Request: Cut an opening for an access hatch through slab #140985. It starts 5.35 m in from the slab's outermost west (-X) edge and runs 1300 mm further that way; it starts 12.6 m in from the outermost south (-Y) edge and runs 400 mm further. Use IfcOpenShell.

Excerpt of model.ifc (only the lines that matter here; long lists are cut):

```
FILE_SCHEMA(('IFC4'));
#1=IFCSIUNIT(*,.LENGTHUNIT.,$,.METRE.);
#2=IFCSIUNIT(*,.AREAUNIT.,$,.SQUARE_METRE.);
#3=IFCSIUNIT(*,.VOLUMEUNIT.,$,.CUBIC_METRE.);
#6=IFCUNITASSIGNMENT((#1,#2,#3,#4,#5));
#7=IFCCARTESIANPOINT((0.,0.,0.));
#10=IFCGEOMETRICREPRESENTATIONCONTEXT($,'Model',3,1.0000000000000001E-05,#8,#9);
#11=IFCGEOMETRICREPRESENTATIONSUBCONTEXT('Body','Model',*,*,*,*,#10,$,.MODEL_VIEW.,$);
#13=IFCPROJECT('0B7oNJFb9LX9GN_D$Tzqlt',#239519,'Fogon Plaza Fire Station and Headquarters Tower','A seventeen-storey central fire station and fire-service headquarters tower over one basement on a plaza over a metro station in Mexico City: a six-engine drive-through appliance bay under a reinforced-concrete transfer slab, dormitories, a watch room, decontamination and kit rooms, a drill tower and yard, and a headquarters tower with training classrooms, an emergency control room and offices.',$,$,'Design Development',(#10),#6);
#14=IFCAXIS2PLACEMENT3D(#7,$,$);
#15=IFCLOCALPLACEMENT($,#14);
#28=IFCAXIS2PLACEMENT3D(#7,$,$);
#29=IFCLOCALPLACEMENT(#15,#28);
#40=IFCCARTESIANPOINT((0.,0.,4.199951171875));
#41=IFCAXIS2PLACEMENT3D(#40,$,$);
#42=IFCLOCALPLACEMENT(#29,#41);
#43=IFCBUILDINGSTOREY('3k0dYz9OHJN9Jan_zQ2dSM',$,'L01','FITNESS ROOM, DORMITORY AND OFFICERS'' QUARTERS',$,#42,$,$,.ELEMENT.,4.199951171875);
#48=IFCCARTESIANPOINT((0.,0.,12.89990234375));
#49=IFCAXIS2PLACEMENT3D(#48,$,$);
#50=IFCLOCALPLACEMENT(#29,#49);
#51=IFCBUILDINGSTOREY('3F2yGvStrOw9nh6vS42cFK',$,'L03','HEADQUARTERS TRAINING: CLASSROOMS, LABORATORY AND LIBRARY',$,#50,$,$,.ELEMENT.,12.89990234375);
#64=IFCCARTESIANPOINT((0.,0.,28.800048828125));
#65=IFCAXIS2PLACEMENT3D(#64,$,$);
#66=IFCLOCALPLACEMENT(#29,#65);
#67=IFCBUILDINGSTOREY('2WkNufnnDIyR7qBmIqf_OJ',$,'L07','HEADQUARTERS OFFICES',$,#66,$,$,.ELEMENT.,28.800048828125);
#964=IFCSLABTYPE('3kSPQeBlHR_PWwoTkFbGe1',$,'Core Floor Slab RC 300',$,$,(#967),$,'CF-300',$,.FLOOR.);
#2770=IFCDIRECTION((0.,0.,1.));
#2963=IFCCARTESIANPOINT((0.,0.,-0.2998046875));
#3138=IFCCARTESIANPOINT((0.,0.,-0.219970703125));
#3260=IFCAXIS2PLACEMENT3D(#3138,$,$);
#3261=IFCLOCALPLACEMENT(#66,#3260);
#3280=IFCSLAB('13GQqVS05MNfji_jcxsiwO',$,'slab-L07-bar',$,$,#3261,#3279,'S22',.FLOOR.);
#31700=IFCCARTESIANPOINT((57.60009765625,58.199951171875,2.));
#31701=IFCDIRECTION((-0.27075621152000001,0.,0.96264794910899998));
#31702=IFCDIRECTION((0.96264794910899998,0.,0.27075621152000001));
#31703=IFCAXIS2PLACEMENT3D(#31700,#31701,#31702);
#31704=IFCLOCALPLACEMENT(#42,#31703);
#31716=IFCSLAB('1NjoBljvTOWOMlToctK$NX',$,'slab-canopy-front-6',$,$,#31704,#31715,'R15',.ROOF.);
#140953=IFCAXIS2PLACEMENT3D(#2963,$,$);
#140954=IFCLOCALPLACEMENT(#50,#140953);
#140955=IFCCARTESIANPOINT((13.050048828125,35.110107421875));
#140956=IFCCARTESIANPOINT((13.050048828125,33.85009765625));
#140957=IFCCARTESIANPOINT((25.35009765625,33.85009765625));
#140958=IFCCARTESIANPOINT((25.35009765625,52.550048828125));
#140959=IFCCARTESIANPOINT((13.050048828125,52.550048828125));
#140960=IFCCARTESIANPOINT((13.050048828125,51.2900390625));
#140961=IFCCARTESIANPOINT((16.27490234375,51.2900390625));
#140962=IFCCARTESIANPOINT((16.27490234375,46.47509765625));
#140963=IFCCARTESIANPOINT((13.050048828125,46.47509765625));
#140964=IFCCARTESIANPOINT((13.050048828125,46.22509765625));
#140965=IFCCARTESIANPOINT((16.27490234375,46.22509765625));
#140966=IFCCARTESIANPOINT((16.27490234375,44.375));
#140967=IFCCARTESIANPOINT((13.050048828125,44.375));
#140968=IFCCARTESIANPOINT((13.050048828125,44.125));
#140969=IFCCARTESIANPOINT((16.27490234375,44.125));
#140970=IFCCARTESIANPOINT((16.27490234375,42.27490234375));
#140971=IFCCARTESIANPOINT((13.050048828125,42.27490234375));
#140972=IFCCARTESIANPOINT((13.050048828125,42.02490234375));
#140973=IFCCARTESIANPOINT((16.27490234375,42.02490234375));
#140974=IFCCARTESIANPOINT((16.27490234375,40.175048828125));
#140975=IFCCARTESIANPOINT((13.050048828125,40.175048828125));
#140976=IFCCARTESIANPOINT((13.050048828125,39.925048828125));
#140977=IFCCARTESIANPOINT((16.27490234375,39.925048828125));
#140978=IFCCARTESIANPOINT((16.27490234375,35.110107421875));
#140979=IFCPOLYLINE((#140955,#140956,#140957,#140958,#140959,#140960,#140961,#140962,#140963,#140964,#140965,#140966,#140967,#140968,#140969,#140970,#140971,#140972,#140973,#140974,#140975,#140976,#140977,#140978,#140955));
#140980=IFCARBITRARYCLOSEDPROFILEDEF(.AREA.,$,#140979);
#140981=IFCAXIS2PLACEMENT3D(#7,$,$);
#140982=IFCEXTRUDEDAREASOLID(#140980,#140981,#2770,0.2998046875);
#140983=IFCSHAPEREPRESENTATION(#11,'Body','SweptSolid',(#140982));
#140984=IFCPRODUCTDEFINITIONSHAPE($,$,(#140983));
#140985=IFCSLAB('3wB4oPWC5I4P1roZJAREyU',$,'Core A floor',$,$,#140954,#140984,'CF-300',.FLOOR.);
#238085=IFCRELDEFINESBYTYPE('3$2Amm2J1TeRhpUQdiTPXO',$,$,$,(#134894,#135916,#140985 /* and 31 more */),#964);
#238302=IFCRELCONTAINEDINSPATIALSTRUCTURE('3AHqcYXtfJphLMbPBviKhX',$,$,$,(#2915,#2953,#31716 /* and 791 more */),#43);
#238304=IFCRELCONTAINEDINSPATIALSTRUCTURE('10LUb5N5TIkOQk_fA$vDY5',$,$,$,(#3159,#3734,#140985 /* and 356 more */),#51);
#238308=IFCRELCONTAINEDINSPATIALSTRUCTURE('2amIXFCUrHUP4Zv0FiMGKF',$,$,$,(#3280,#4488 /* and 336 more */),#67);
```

```python
import numpy as np
import ifcopenshell
import ifcopenshell.api.feature
import ifcopenshell.api.geometry
import ifcopenshell.api.root
import ifcopenshell.geom
import ifcopenshell.util.placement
import ifcopenshell.util.representation
import ifcopenshell.util.shape
import ifcopenshell.util.unit

model = ifcopenshell.open("model.ifc")
unit_scale = ifcopenshell.util.unit.calculate_unit_scale(model)
settings = ifcopenshell.geom.settings()


def volume(element):
    """Net volume in cubic metres, openings subtracted."""
    shape = ifcopenshell.geom.create_shape(settings, element)
    return ifcopenshell.util.shape.get_volume(shape.geometry)


slab = model.by_guid("3wB4oPWC5I4P1roZJAREyU")
before = volume(slab)

# Extent in the slab's own axes, in metres. The edges named are its -X and -Y sides.
slab_shape = ifcopenshell.geom.create_shape(settings, slab)
vertices = ifcopenshell.util.shape.get_vertices(slab_shape.geometry)
x_min, y_min, bottom = vertices.min(axis=0)
top = vertices[:, 2].max()

opening = ifcopenshell.api.root.create_entity(model, ifc_class="IfcOpeningElement", name="Access hatch opening", predefined_type="OPENING")
context = ifcopenshell.util.representation.get_context(model, "Model", "Body", "MODEL_VIEW")
width, depth = 1.3, 0.4
outline = [(0.0, 0.0), (width, 0.0), (width, depth), (0.0, depth), (0.0, 0.0)]
# Overshoot both faces by 50 mm so the cut is clean.
shape = ifcopenshell.api.geometry.add_slab_representation(
    model, context=context, depth=top - bottom + 0.1, polyline=outline
)
ifcopenshell.api.geometry.assign_representation(model, product=opening, representation=shape)

matrix = ifcopenshell.util.placement.get_local_placement(slab.ObjectPlacement)
matrix[:, 3] = matrix @ np.append(np.array([x_min + 5.35, y_min + 12.6, bottom - 0.05]) / unit_scale, 1.0)
ifcopenshell.api.geometry.edit_object_placement(model, product=opening, matrix=matrix, is_si=False)
ifcopenshell.api.feature.add_feature(model, feature=opening, element=slab)

after = volume(slab)

print(f"slab volume {before:.3f} -> {after:.3f} m3")

model.write("model-out.ifc")
```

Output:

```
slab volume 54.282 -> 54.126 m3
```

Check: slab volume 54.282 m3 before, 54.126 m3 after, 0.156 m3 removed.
